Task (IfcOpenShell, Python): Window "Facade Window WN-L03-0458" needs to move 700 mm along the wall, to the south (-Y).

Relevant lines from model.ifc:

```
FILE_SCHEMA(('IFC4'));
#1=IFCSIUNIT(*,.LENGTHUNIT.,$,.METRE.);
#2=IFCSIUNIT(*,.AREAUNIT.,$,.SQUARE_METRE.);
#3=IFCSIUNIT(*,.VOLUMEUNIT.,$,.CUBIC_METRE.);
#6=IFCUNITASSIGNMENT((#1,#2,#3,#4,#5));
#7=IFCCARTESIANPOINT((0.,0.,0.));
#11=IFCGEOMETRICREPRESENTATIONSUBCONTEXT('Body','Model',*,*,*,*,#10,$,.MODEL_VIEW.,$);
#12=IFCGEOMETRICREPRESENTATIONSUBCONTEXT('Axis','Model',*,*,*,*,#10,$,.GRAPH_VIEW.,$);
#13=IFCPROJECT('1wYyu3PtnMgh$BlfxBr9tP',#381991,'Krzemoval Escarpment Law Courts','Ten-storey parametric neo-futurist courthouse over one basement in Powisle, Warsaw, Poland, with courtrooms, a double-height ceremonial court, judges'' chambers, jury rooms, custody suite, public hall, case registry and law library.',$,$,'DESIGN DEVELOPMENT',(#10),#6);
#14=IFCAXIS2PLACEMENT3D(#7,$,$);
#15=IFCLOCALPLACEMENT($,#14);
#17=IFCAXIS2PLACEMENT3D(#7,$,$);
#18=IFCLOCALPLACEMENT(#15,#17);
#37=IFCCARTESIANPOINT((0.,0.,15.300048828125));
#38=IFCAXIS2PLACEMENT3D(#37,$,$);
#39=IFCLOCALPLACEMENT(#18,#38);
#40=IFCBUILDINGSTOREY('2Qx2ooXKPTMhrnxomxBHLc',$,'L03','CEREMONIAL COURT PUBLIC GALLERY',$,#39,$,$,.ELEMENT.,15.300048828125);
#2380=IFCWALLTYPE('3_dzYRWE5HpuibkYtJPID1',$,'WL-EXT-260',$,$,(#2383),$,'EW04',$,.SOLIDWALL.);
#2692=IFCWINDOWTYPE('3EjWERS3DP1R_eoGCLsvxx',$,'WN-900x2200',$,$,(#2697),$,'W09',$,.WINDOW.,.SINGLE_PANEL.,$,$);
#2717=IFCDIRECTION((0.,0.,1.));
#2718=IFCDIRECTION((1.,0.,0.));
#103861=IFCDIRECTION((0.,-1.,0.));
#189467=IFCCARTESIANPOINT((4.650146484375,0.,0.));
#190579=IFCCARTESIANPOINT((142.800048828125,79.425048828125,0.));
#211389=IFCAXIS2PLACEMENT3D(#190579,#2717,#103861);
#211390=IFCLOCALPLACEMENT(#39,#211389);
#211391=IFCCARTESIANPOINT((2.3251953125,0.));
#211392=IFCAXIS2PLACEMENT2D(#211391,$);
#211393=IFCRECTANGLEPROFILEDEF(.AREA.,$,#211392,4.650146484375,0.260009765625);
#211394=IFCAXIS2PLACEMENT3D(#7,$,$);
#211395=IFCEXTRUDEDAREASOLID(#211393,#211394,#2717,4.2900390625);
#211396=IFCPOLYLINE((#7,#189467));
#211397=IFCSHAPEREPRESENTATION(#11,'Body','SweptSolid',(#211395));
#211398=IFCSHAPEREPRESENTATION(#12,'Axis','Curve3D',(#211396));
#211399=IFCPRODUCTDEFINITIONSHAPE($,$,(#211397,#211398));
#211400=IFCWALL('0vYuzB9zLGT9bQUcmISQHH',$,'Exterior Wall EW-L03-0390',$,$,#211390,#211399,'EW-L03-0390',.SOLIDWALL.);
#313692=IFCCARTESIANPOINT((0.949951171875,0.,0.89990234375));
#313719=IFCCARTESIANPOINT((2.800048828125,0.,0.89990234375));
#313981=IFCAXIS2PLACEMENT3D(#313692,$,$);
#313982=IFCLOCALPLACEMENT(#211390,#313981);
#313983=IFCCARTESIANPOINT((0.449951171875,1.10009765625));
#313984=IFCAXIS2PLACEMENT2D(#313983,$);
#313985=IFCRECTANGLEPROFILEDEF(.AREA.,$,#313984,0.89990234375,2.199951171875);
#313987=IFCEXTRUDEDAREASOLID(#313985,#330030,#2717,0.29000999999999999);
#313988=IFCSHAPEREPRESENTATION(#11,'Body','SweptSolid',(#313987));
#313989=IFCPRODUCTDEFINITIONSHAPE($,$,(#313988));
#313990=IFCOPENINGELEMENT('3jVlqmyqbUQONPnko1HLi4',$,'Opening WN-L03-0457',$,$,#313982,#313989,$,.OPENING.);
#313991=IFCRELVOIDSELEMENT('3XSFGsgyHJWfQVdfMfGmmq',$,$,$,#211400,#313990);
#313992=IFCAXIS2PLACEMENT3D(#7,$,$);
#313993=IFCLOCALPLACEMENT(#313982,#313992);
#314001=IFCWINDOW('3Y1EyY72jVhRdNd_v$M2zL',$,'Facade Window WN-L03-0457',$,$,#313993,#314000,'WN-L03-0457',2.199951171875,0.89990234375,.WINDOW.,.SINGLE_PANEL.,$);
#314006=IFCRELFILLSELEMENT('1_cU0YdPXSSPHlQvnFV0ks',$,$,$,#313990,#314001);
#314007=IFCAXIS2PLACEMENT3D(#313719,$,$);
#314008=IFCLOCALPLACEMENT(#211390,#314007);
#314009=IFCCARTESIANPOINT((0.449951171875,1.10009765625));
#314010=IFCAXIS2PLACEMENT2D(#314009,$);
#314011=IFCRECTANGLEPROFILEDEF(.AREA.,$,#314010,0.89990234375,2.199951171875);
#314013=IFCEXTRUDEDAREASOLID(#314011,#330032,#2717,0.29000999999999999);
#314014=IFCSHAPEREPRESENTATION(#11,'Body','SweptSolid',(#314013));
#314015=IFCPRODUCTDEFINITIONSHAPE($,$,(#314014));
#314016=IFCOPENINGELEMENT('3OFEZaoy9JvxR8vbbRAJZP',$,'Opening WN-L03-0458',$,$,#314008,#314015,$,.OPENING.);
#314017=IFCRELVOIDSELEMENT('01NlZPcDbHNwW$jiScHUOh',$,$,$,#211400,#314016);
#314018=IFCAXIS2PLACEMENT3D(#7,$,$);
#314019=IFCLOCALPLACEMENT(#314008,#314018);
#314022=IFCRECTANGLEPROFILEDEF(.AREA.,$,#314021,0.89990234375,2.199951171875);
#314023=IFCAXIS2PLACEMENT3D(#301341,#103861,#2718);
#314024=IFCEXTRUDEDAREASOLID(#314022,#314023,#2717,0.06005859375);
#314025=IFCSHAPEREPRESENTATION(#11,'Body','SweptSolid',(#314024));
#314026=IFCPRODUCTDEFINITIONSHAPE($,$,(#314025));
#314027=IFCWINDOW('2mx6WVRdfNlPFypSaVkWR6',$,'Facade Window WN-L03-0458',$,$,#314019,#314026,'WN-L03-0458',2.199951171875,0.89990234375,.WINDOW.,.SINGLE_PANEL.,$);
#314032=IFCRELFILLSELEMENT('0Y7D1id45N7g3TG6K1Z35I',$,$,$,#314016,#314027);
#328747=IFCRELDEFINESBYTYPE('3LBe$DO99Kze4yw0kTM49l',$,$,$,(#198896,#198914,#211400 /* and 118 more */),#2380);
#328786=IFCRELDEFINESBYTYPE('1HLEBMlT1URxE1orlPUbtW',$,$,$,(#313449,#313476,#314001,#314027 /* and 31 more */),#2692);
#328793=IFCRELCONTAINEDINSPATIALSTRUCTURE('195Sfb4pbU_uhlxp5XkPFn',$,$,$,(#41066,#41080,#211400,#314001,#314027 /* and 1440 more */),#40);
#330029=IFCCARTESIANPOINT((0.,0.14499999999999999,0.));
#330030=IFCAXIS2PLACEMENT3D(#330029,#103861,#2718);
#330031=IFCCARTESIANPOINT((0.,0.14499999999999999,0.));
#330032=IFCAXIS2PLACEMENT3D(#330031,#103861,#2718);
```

```python
import ifcopenshell
import ifcopenshell.api.geometry
import ifcopenshell.util.placement
import ifcopenshell.util.unit

model = ifcopenshell.open("model.ifc")
unit_scale = ifcopenshell.util.unit.calculate_unit_scale(model)

window = model.by_id(314027)
opening = window.FillsVoids[0].RelatingOpeningElement
wall = opening.VoidsElements[0].RelatingBuildingElement

wall_matrix = ifcopenshell.util.placement.get_local_placement(wall.ObjectPlacement)
shift = wall_matrix[:3, 0] * 0.7 / unit_scale
before = ifcopenshell.util.placement.get_local_placement(window.ObjectPlacement)[:3, 3].copy()

# The window is placed relative to its opening, so it follows when the opening moves.
matrix = ifcopenshell.util.placement.get_local_placement(opening.ObjectPlacement)
matrix[:3, 3] += shift
ifcopenshell.api.geometry.edit_object_placement(
    model, product=opening, matrix=matrix, is_si=False, should_transform_children=True
)

after = ifcopenshell.util.placement.get_local_placement(window.ObjectPlacement)[:3, 3]
print("window moved by", (after - before).round(3) + 0.0)

model.write("model-out.ifc")
```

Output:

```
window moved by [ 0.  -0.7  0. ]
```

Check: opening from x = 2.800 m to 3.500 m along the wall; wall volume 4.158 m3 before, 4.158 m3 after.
